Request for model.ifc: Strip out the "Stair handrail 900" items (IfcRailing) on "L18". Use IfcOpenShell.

First a look at what the model holds.

```python
import ifcopenshell
import ifcopenshell.util.element

model = ifcopenshell.open("model.ifc")
print(model.schema)
storey = next(s for s in model.by_type("IfcBuildingStorey") if s.Name == "L18")
railings = [e for e in ifcopenshell.util.element.get_decomposition(storey) if e.is_a("IfcRailing")]
seen = {}
for e in railings:
    element_type = ifcopenshell.util.element.get_type(e)
    name = element_type.Name if element_type not in (None, e) else None
    seen[name] = seen.get(name, 0) + 1
for name, count in sorted(seen.items(), key=str):
    print(count, "x", name)
```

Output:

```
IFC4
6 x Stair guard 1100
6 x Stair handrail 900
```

```python
import ifcopenshell
import ifcopenshell.api.root
import ifcopenshell.util.element

model = ifcopenshell.open("model.ifc")

storey = next(s for s in model.by_type("IfcBuildingStorey") if s.Name == "L18")
railings = [e for e in ifcopenshell.util.element.get_decomposition(storey) if e.is_a("IfcRailing")]
targets = [e for e in railings if (t := ifcopenshell.util.element.get_type(e)) not in (None, e) and t.Name == "Stair handrail 900"]

for e in targets:
    ifcopenshell.api.root.remove_product(model, product=e)
print(len(targets), "removed")

model.write("model-out.ifc")
```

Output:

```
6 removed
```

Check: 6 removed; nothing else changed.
